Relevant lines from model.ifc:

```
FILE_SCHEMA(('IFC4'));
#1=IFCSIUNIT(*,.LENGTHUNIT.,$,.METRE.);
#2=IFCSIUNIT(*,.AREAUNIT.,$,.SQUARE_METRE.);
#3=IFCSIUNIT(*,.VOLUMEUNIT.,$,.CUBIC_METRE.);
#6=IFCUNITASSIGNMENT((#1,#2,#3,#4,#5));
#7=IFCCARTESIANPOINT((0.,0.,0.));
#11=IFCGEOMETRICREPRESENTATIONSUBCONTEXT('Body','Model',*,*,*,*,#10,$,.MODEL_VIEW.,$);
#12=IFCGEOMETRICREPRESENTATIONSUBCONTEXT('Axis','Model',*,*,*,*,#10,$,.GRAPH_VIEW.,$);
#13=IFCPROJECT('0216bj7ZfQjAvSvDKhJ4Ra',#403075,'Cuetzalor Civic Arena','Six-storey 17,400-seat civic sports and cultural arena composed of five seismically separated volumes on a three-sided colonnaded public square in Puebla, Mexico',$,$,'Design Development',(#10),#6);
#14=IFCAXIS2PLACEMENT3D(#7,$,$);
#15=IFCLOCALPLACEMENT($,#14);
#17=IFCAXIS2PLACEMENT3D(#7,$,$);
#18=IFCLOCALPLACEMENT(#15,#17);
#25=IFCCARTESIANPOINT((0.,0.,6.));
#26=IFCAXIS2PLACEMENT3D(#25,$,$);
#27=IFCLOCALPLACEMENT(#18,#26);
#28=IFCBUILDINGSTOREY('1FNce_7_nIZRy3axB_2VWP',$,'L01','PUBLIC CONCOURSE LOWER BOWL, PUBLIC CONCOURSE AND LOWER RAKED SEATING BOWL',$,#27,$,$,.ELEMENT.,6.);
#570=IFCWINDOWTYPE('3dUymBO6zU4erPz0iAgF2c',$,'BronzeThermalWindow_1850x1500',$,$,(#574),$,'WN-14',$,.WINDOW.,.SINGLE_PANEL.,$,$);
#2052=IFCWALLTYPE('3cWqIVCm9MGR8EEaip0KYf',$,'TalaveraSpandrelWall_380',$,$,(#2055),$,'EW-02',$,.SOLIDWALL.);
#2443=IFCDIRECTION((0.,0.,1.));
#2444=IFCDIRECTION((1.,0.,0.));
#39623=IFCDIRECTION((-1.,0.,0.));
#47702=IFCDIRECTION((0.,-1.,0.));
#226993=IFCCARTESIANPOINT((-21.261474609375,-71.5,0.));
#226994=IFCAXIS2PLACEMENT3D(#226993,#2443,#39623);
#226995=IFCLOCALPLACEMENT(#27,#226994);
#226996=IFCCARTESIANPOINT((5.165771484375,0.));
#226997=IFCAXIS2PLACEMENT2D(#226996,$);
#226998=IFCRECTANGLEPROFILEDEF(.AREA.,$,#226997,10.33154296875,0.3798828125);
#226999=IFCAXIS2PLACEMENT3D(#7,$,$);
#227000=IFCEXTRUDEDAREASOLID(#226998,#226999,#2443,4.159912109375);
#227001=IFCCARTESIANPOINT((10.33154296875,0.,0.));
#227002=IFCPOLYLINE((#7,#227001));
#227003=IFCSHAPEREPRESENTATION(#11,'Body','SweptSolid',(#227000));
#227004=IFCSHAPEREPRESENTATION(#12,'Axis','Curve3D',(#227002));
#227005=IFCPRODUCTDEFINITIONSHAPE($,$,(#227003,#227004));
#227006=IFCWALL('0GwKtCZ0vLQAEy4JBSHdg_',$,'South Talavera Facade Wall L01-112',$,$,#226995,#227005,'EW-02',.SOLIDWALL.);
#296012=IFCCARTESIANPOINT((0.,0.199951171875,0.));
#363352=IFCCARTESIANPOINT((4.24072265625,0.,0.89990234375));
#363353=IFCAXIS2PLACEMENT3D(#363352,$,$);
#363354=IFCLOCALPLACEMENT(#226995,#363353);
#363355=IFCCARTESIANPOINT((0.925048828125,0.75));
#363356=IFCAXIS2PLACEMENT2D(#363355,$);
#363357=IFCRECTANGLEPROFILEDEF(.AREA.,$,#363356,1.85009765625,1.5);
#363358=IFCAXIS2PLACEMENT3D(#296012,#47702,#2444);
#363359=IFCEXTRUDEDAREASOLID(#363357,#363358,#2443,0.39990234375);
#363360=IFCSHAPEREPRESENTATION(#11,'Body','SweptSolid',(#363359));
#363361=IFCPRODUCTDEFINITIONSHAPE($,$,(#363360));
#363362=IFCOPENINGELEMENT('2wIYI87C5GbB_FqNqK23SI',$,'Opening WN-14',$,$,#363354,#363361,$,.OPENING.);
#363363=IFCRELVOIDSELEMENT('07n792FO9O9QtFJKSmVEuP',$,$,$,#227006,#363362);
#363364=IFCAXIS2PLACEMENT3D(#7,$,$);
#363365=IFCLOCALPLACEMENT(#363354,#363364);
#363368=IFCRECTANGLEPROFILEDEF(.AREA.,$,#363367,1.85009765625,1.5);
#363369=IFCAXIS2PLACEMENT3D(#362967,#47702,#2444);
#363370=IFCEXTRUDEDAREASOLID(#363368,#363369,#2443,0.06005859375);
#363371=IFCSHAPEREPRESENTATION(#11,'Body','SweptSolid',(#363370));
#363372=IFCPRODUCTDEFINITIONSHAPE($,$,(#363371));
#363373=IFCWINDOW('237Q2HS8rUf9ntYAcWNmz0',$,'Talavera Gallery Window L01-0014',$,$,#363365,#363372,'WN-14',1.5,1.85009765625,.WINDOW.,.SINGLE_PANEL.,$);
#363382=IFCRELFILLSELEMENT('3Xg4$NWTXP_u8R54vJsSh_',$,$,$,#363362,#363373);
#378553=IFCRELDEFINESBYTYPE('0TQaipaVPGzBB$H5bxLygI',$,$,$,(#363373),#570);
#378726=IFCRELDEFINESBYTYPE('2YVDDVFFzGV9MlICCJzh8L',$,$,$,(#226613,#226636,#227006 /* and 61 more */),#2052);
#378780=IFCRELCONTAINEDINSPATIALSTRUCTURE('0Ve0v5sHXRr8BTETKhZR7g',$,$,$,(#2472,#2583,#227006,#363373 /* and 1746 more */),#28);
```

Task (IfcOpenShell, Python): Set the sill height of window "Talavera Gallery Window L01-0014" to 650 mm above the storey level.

```python
import numpy as np
import ifcopenshell
import ifcopenshell.api.geometry
import ifcopenshell.geom
import ifcopenshell.util.element
import ifcopenshell.util.placement
import ifcopenshell.util.shape
import ifcopenshell.util.unit

model = ifcopenshell.open("model.ifc")
unit_scale = ifcopenshell.util.unit.calculate_unit_scale(model)

window = model.by_id(363373)
opening = window.FillsVoids[0].RelatingOpeningElement
storey = ifcopenshell.util.element.get_container(window, ifc_class="IfcBuildingStorey")
level = ifcopenshell.util.placement.get_local_placement(storey.ObjectPlacement)[2, 3]

# The opening's origin need not be at the sill, so measure its lowest point.
shape = ifcopenshell.geom.create_shape(ifcopenshell.geom.settings(), opening)
bottom = ifcopenshell.util.shape.get_shape_bottom_elevation(shape, shape.geometry) / unit_scale
dz = level + 0.65 / unit_scale - bottom

shift = np.array([0.0, 0.0, dz])
# The window is placed relative to its opening, so it follows when the opening moves.
matrix = ifcopenshell.util.placement.get_local_placement(opening.ObjectPlacement)
matrix[:3, 3] += shift
ifcopenshell.api.geometry.edit_object_placement(
    model, product=opening, matrix=matrix, is_si=False, should_transform_children=True
)

print(f"moved by {dz * unit_scale:+.3f} m")

model.write("model_v2.ifc")
```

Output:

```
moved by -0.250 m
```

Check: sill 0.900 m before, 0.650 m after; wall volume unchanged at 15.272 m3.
